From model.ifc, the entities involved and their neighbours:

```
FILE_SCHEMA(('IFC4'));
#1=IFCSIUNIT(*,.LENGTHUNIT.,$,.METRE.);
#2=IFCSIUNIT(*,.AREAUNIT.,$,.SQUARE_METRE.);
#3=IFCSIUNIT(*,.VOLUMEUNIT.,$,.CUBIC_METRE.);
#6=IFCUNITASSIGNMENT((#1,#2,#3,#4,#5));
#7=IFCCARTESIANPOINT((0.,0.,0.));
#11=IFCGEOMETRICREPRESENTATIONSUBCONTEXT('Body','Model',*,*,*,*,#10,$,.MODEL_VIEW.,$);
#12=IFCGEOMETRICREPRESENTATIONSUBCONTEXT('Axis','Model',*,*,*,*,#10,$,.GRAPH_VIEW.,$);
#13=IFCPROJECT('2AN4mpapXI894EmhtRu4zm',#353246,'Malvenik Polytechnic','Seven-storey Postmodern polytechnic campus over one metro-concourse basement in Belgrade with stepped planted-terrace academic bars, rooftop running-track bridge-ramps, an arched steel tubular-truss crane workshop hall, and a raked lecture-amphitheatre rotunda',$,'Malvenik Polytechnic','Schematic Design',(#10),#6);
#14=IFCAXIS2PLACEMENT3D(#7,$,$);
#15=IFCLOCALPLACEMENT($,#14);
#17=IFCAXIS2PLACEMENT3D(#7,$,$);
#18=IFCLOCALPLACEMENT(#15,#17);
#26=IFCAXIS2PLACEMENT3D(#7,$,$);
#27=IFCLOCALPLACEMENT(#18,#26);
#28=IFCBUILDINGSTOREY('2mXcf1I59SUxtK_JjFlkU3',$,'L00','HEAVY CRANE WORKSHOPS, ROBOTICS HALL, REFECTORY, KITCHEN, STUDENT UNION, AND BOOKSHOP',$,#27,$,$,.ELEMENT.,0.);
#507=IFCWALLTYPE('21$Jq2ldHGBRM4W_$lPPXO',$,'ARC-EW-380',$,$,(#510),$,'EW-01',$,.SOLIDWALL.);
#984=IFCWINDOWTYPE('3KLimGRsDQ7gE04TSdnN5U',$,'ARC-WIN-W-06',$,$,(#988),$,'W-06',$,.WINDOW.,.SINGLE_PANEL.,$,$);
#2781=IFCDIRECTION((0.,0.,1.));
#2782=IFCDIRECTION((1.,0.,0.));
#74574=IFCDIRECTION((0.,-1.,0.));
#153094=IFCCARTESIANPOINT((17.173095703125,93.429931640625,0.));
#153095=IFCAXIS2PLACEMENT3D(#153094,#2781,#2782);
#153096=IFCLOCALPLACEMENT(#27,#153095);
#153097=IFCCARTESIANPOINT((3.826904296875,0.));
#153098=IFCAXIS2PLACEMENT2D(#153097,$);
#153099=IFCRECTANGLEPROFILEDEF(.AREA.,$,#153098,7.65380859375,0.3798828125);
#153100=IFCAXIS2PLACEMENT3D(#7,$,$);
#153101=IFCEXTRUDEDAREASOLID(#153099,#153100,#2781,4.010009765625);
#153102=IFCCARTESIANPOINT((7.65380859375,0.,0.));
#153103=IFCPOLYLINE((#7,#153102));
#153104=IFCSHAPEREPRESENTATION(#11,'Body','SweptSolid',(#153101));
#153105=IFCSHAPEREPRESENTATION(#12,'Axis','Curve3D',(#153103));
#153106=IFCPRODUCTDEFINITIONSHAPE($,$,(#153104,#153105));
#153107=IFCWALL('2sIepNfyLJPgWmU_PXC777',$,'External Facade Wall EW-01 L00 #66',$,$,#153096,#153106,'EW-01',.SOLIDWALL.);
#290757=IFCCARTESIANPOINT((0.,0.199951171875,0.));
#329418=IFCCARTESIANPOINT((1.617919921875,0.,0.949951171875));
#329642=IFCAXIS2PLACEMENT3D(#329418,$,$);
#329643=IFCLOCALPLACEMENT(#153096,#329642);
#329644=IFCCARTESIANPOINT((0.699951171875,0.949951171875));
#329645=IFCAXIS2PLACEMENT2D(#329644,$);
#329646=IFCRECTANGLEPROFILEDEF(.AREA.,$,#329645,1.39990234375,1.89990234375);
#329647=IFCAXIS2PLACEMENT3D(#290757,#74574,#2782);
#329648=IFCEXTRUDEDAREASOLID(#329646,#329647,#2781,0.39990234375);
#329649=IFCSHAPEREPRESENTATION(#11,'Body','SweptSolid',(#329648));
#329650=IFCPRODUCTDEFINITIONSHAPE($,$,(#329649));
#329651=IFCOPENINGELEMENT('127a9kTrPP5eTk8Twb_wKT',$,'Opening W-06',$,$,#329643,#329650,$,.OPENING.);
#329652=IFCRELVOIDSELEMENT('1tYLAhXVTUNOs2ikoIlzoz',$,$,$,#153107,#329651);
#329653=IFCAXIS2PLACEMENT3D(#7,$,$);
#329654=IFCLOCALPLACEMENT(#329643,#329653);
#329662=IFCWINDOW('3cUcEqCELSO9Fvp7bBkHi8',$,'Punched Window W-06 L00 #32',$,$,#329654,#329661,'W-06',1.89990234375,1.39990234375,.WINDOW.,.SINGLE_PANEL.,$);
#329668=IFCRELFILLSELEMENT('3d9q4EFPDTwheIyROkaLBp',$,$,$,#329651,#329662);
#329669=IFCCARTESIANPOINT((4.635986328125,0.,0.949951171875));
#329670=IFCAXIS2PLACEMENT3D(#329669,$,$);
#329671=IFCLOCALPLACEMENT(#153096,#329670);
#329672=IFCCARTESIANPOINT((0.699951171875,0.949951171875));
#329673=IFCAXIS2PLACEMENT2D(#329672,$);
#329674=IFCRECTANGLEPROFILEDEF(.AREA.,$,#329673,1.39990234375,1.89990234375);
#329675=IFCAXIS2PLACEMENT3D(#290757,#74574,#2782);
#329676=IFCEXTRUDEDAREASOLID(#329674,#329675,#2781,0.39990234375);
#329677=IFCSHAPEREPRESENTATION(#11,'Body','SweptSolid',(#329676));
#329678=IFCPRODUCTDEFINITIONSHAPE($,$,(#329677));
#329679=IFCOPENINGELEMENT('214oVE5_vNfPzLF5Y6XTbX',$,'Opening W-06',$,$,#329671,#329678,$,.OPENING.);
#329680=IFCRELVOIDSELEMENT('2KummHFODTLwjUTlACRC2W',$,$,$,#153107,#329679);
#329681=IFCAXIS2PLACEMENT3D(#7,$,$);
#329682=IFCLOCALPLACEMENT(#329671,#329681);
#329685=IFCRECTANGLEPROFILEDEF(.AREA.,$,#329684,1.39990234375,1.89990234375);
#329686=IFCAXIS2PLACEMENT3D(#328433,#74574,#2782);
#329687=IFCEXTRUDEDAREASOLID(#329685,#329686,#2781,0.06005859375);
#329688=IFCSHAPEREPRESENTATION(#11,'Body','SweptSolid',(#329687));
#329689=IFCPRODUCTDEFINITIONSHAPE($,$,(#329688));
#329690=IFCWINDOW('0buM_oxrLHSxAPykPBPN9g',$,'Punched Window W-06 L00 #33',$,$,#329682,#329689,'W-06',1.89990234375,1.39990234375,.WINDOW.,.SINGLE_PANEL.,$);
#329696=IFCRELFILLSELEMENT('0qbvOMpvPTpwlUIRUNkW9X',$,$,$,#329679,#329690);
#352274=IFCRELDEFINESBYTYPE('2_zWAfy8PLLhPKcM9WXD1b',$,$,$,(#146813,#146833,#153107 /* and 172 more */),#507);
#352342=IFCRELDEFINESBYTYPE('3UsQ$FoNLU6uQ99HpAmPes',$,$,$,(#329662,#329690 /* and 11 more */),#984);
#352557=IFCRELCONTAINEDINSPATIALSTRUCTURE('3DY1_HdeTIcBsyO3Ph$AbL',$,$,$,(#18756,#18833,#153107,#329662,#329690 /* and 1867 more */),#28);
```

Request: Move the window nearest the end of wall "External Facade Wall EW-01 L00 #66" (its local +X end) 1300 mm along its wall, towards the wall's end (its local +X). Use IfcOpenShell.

```python
import ifcopenshell
import ifcopenshell.api.geometry
import ifcopenshell.util.placement
import ifcopenshell.util.unit

model = ifcopenshell.open("model.ifc")
unit_scale = ifcopenshell.util.unit.calculate_unit_scale(model)

window = model.by_guid("0buM_oxrLHSxAPykPBPN9g")
opening = window.FillsVoids[0].RelatingOpeningElement
wall = opening.VoidsElements[0].RelatingBuildingElement

wall_matrix = ifcopenshell.util.placement.get_local_placement(wall.ObjectPlacement)
shift = wall_matrix[:3, 0] * 1.3 / unit_scale
before = ifcopenshell.util.placement.get_local_placement(window.ObjectPlacement)[:3, 3].copy()

# The window is placed relative to its opening, so it follows when the opening moves.
matrix = ifcopenshell.util.placement.get_local_placement(opening.ObjectPlacement)
matrix[:3, 3] += shift
ifcopenshell.api.geometry.edit_object_placement(
    model, product=opening, matrix=matrix, is_si=False, should_transform_children=True
)

after = ifcopenshell.util.placement.get_local_placement(window.ObjectPlacement)[:3, 3]
print("window moved by", (after - before).round(3) + 0.0)

model.write("model_rev.ifc")
```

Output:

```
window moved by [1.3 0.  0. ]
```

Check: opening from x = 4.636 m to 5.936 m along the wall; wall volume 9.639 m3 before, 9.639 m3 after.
